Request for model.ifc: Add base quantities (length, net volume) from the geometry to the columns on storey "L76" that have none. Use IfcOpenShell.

First a look at what the model holds.

```python
import ifcopenshell
import ifcopenshell.util.element
import ifcopenshell.util.unit

model = ifcopenshell.open("model.ifc")
print(model.schema)
for unit_type in ("LENGTHUNIT", "AREAUNIT", "VOLUMEUNIT"):
    print(unit_type, ifcopenshell.util.unit.calculate_unit_scale(model, unit_type))
storey = next(s for s in model.by_type("IfcBuildingStorey") if s.Name == "L76")
columns = [e for e in ifcopenshell.util.element.get_decomposition(storey) if e.is_a("IfcColumn")]
for e in sorted(columns, key=lambda e: e.id()):
    print(e.id(), e.is_a(), e.Name, list(ifcopenshell.util.element.get_psets(e, qtos_only=True)), sep=" | ")
```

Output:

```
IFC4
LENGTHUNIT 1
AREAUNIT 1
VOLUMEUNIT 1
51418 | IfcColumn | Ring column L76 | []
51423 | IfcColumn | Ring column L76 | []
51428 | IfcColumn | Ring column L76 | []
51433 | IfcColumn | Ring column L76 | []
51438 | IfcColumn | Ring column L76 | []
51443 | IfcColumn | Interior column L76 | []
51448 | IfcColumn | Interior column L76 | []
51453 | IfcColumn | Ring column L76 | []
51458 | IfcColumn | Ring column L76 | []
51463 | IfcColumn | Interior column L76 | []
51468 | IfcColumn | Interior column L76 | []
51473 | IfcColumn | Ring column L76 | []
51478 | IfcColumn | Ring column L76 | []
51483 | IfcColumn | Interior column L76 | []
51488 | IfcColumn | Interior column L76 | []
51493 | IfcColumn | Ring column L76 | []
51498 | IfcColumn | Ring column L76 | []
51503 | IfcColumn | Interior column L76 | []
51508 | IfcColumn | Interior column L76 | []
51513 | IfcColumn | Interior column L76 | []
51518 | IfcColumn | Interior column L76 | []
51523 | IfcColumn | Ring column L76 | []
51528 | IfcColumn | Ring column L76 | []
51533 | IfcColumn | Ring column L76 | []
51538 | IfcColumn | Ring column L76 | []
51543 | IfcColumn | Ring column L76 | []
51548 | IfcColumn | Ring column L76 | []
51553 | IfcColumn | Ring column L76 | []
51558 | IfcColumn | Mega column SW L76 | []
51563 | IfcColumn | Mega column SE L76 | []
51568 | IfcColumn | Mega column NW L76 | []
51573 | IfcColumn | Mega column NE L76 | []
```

```python
import ifcopenshell
import ifcopenshell.api.pset
import ifcopenshell.geom
import ifcopenshell.util.element
import ifcopenshell.util.shape
import ifcopenshell.util.unit

model = ifcopenshell.open("model.ifc")
unit_scale = ifcopenshell.util.unit.calculate_unit_scale(model)
volume_scale = ifcopenshell.util.unit.calculate_unit_scale(model, "VOLUMEUNIT")
settings = ifcopenshell.geom.settings()

storey = next(s for s in model.by_type("IfcBuildingStorey") if s.Name == "L76")
columns = [e for e in ifcopenshell.util.element.get_decomposition(storey) if e.is_a("IfcColumn")]

for e in sorted(columns, key=lambda e: e.id()):
    if ifcopenshell.util.element.get_psets(e, qtos_only=True, should_inherit=False):
        continue
    # Geometry comes back in metres, in the element's own axes.
    shape = ifcopenshell.geom.create_shape(settings, e)
    values = {
        "Length": ifcopenshell.util.shape.get_z(shape.geometry) / unit_scale,
        "NetVolume": ifcopenshell.util.shape.get_volume(shape.geometry) / volume_scale,
    }
    qto = ifcopenshell.api.pset.add_qto(model, product=e, name="Qto_ColumnBaseQuantities")
    ifcopenshell.api.pset.edit_qto(model, qto=qto, properties=values)
    print(e.id(), {k: round(v, 3) for k, v in values.items()})

model.write("model_updated.ifc")
```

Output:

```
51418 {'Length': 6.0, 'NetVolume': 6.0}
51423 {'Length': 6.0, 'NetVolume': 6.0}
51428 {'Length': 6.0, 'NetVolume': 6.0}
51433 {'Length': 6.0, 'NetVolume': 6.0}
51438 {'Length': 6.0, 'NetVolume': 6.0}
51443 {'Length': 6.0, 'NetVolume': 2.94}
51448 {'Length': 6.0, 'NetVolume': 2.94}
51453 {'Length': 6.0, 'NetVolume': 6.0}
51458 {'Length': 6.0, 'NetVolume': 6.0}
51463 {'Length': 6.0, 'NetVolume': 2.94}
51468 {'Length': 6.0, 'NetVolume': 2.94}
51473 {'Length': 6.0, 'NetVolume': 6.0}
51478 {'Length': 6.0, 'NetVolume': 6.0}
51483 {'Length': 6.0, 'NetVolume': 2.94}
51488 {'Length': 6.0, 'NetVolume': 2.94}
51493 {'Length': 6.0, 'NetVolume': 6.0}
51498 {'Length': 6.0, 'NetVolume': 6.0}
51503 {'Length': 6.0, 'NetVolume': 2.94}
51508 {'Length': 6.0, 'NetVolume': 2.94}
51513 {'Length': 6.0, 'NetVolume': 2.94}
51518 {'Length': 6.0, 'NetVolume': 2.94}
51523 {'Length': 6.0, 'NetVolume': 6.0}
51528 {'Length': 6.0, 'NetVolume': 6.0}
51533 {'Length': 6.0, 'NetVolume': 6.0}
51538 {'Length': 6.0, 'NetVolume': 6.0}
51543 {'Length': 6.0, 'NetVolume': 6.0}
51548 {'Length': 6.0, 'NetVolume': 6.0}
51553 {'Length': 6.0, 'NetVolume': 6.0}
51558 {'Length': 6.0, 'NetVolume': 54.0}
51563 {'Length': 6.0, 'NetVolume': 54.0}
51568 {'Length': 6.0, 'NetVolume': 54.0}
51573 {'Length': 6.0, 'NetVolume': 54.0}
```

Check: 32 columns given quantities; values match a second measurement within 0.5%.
